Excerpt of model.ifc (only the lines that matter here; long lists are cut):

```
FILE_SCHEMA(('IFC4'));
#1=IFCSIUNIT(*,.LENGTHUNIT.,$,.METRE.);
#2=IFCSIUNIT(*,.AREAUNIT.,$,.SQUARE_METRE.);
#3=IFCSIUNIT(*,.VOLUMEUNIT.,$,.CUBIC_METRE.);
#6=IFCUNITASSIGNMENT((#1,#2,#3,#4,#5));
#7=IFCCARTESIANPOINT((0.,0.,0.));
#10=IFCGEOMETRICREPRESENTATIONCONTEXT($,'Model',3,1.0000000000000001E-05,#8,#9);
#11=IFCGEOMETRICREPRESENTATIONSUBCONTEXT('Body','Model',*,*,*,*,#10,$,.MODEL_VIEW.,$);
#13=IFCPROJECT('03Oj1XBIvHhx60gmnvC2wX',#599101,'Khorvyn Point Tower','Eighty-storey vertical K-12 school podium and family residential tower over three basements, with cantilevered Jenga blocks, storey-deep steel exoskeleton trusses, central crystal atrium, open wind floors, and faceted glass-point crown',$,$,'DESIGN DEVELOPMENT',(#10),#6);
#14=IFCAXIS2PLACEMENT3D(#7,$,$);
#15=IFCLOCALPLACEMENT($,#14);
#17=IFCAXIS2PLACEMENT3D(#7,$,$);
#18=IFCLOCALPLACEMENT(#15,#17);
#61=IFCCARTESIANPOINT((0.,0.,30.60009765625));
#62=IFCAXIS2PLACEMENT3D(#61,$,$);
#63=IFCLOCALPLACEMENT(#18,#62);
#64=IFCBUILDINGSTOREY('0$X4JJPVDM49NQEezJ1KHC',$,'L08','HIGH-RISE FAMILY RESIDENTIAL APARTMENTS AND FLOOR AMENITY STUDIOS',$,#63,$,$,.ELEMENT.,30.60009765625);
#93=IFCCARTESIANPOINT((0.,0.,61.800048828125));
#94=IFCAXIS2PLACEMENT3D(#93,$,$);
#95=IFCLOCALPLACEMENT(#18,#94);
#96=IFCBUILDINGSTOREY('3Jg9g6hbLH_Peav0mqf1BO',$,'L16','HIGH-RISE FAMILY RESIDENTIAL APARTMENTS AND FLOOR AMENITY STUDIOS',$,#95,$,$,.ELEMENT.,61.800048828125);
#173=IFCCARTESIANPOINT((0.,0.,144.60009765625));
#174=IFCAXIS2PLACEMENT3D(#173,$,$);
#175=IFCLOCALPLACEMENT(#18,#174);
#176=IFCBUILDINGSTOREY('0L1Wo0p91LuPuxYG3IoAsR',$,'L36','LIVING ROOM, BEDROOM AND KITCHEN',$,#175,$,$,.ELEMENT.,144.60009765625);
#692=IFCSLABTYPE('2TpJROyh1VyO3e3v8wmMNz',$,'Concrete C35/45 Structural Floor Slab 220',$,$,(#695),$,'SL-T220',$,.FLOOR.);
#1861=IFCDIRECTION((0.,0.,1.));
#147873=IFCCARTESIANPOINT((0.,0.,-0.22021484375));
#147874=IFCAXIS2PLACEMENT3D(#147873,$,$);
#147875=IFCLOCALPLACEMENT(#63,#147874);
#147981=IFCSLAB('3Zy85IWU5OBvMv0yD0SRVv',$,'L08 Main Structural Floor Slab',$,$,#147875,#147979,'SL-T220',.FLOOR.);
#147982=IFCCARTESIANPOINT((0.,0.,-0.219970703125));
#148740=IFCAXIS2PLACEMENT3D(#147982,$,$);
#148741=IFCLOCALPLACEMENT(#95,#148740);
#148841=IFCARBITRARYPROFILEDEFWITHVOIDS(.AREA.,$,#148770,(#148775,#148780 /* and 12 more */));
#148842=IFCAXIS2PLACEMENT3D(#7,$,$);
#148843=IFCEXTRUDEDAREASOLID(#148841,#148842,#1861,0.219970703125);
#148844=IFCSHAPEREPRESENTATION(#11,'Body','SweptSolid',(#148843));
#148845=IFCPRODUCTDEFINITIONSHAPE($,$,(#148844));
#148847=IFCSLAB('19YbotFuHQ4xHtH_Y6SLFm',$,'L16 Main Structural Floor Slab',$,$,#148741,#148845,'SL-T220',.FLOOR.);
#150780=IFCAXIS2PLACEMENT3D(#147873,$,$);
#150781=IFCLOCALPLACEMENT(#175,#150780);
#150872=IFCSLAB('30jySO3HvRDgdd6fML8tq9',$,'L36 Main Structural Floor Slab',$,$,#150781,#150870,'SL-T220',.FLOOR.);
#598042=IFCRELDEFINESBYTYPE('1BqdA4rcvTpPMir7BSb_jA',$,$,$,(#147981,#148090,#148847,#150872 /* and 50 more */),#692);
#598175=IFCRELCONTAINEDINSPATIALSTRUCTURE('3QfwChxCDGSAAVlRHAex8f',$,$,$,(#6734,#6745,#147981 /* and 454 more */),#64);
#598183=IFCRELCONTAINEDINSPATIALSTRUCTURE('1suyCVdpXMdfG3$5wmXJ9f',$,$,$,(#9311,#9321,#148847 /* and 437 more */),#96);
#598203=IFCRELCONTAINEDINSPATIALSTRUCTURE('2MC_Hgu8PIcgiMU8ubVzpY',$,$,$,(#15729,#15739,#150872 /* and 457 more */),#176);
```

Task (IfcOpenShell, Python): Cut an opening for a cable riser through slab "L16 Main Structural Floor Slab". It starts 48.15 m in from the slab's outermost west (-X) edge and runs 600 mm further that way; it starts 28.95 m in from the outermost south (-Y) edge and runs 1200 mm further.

```python
import numpy as np
import ifcopenshell
import ifcopenshell.api.feature
import ifcopenshell.api.geometry
import ifcopenshell.api.root
import ifcopenshell.geom
import ifcopenshell.util.placement
import ifcopenshell.util.representation
import ifcopenshell.util.shape
import ifcopenshell.util.unit

model = ifcopenshell.open("model.ifc")
unit_scale = ifcopenshell.util.unit.calculate_unit_scale(model)
settings = ifcopenshell.geom.settings()


def volume(element):
    """Net volume in cubic metres, openings subtracted."""
    shape = ifcopenshell.geom.create_shape(settings, element)
    return ifcopenshell.util.shape.get_volume(shape.geometry)


slab = model.by_id(148847)
before = volume(slab)

# Extent in the slab's own axes, in metres. The edges named are its -X and -Y sides.
slab_shape = ifcopenshell.geom.create_shape(settings, slab)
vertices = ifcopenshell.util.shape.get_vertices(slab_shape.geometry)
x_min, y_min, bottom = vertices.min(axis=0)
top = vertices[:, 2].max()

opening = ifcopenshell.api.root.create_entity(model, ifc_class="IfcOpeningElement", name="Cable riser opening", predefined_type="OPENING")
context = ifcopenshell.util.representation.get_context(model, "Model", "Body", "MODEL_VIEW")
width, depth = 0.6, 1.2
outline = [(0.0, 0.0), (width, 0.0), (width, depth), (0.0, depth), (0.0, 0.0)]
# Overshoot both faces by 50 mm so the cut is clean.
shape = ifcopenshell.api.geometry.add_slab_representation(
    model, context=context, depth=top - bottom + 0.1, polyline=outline
)
ifcopenshell.api.geometry.assign_representation(model, product=opening, representation=shape)

matrix = ifcopenshell.util.placement.get_local_placement(slab.ObjectPlacement)
matrix[:, 3] = matrix @ np.append(np.array([x_min + 48.15, y_min + 28.95, bottom - 0.05]) / unit_scale, 1.0)
ifcopenshell.api.geometry.edit_object_placement(model, product=opening, matrix=matrix, is_si=False)
ifcopenshell.api.feature.add_feature(model, feature=opening, element=slab)

after = volume(slab)

print(f"slab volume {before:.3f} -> {after:.3f} m3")

model.write("model_rev.ifc")
```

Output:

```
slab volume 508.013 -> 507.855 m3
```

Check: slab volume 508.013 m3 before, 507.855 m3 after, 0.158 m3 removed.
